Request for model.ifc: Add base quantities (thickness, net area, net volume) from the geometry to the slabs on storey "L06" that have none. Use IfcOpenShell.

First a look at what the model holds.

```python
import ifcopenshell
import ifcopenshell.util.element
import ifcopenshell.util.unit

model = ifcopenshell.open("model.ifc")
print(model.schema)
for unit_type in ("LENGTHUNIT", "AREAUNIT", "VOLUMEUNIT"):
    print(unit_type, ifcopenshell.util.unit.calculate_unit_scale(model, unit_type))
storey = next(s for s in model.by_type("IfcBuildingStorey") if s.Name == "L06")
slabs = [e for e in ifcopenshell.util.element.get_decomposition(storey) if e.is_a("IfcSlab")]
for e in sorted(slabs, key=lambda e: e.id()):
    print(e.id(), e.is_a(), e.Name, list(ifcopenshell.util.element.get_psets(e, qtos_only=True)), sep=" | ")
```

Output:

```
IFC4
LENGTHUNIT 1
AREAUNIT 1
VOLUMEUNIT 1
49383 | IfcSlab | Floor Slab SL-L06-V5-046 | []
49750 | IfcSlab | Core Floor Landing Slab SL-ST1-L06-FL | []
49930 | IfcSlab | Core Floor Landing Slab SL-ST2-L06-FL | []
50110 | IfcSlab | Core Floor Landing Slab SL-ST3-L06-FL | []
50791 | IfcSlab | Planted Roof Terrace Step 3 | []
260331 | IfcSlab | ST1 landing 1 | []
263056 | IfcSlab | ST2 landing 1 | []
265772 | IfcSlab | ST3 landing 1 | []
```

```python
import ifcopenshell
import ifcopenshell.api.pset
import ifcopenshell.geom
import ifcopenshell.util.element
import ifcopenshell.util.shape
import ifcopenshell.util.unit

model = ifcopenshell.open("model.ifc")
unit_scale = ifcopenshell.util.unit.calculate_unit_scale(model)
area_scale = ifcopenshell.util.unit.calculate_unit_scale(model, "AREAUNIT")
volume_scale = ifcopenshell.util.unit.calculate_unit_scale(model, "VOLUMEUNIT")
settings = ifcopenshell.geom.settings()

storey = next(s for s in model.by_type("IfcBuildingStorey") if s.Name == "L06")
slabs = [e for e in ifcopenshell.util.element.get_decomposition(storey) if e.is_a("IfcSlab")]

for e in sorted(slabs, key=lambda e: e.id()):
    if ifcopenshell.util.element.get_psets(e, qtos_only=True, should_inherit=False):
        continue
    # Geometry comes back in metres, in the element's own axes.
    shape = ifcopenshell.geom.create_shape(settings, e)
    values = {
        "Width": ifcopenshell.util.shape.get_z(shape.geometry) / unit_scale,
        "NetArea": ifcopenshell.util.shape.get_footprint_area(shape.geometry) / area_scale,
        "NetVolume": ifcopenshell.util.shape.get_volume(shape.geometry) / volume_scale,
    }
    qto = ifcopenshell.api.pset.add_qto(model, product=e, name="Qto_SlabBaseQuantities")
    ifcopenshell.api.pset.edit_qto(model, qto=qto, properties=values)
    print(e.id(), {k: round(v, 3) for k, v in values.items()})

model.write("model_rev.ifc")
```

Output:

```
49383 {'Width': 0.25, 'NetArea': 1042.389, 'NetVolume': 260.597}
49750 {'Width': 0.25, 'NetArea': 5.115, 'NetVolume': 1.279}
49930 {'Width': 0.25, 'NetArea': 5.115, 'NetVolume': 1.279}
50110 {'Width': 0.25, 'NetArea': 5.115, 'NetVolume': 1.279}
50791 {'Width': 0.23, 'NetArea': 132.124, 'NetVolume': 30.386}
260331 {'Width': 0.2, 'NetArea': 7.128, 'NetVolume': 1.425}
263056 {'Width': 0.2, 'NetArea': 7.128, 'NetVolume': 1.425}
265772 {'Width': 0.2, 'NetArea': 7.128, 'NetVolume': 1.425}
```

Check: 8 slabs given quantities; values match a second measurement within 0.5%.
